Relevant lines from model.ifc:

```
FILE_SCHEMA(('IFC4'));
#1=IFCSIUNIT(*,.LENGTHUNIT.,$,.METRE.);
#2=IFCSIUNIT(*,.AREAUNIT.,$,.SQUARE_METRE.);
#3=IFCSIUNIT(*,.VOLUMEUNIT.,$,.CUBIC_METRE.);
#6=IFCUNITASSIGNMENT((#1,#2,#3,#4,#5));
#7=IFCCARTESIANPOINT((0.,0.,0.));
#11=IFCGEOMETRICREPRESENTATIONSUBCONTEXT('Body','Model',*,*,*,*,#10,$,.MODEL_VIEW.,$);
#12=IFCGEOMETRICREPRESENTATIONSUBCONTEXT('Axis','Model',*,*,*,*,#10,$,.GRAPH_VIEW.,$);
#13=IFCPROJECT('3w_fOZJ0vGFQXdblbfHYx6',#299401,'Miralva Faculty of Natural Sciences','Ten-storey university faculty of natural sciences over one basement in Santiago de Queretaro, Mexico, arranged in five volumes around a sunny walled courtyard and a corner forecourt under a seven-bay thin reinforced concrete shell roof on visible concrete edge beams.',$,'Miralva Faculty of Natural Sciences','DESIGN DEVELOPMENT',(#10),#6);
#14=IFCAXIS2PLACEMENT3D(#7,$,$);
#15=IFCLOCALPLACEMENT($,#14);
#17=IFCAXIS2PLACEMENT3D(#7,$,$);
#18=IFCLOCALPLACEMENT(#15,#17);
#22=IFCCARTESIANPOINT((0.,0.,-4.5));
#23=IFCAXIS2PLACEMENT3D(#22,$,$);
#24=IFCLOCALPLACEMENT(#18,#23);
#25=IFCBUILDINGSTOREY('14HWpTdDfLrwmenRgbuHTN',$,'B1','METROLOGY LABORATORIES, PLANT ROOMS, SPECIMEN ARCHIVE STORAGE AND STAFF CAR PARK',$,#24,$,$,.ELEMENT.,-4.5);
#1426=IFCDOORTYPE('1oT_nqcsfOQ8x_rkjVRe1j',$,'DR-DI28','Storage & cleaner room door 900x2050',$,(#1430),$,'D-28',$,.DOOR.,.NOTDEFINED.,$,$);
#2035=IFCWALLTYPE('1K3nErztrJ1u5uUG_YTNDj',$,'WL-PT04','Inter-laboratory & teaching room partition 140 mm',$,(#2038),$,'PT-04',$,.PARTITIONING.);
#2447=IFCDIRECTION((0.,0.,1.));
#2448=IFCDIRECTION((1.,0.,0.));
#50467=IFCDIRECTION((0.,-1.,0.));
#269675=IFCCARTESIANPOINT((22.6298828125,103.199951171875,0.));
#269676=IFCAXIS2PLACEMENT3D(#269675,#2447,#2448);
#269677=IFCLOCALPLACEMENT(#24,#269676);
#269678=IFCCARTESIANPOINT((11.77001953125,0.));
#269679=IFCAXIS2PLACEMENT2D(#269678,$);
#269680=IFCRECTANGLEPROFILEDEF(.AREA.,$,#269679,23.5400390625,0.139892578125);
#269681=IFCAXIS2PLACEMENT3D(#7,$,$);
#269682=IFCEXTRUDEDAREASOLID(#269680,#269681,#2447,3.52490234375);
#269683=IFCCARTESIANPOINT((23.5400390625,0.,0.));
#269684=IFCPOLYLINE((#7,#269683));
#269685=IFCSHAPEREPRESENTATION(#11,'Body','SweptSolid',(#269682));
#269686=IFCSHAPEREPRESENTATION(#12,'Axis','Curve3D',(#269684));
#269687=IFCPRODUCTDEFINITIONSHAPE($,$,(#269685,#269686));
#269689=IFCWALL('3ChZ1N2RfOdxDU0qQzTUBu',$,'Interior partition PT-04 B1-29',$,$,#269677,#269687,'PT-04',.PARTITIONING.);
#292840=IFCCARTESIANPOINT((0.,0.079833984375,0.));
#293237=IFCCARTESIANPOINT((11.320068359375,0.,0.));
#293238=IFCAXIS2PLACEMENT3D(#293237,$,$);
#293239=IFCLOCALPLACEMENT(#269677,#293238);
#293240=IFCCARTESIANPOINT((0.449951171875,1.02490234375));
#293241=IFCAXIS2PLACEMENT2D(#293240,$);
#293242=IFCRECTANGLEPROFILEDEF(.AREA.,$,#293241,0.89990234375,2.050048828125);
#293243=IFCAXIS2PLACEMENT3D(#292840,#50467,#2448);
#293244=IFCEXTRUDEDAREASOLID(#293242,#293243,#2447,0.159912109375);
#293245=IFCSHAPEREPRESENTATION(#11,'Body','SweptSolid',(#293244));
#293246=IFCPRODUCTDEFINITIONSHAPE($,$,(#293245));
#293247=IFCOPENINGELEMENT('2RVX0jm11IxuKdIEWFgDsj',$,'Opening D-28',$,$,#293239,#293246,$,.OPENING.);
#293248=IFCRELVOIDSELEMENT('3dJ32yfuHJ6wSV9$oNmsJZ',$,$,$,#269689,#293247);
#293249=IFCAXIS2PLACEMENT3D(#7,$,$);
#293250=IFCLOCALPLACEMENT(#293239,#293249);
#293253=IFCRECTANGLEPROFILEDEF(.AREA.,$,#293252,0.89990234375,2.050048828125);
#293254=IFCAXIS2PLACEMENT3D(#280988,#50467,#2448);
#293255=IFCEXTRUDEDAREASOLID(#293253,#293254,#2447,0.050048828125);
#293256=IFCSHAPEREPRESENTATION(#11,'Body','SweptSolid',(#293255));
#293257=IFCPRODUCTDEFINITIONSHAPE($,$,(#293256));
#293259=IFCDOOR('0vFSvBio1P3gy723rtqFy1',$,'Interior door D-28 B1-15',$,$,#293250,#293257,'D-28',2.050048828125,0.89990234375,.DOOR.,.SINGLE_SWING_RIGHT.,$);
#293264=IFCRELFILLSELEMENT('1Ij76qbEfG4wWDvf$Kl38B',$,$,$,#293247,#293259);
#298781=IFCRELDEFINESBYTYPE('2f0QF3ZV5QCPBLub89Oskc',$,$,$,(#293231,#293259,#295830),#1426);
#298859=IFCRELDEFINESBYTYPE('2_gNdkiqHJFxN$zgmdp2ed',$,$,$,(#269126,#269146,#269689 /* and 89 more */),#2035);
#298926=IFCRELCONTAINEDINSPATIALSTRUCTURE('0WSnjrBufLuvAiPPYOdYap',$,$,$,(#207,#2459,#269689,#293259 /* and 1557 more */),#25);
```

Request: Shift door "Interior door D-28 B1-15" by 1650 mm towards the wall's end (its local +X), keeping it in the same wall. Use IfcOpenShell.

```python
import ifcopenshell
import ifcopenshell.api.geometry
import ifcopenshell.util.placement
import ifcopenshell.util.unit

model = ifcopenshell.open("model.ifc")
unit_scale = ifcopenshell.util.unit.calculate_unit_scale(model)

door = model.by_guid("0vFSvBio1P3gy723rtqFy1")
opening = door.FillsVoids[0].RelatingOpeningElement
wall = opening.VoidsElements[0].RelatingBuildingElement

wall_matrix = ifcopenshell.util.placement.get_local_placement(wall.ObjectPlacement)
shift = wall_matrix[:3, 0] * 1.65 / unit_scale
before = ifcopenshell.util.placement.get_local_placement(door.ObjectPlacement)[:3, 3].copy()

# The door is placed relative to its opening, so it follows when the opening moves.
matrix = ifcopenshell.util.placement.get_local_placement(opening.ObjectPlacement)
matrix[:3, 3] += shift
ifcopenshell.api.geometry.edit_object_placement(
    model, product=opening, matrix=matrix, is_si=False, should_transform_children=True
)

after = ifcopenshell.util.placement.get_local_placement(door.ObjectPlacement)[:3, 3]
print("door moved by", (after - before).round(3) + 0.0)

model.write("model-out.ifc")
```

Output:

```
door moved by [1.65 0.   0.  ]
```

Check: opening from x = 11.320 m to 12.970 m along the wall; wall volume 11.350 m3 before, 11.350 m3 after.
